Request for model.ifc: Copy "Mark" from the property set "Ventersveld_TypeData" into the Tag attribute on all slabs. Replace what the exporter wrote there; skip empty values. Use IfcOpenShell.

First a look at what the model holds.

```python
import ifcopenshell
import ifcopenshell.util.element

model = ifcopenshell.open("model.ifc")
print(model.schema)
slabs = model.by_type("IfcSlab")
print(len(slabs), "slabs")
for e in slabs[:8]:
    source = ifcopenshell.util.element.get_pset(e, "Ventersveld_TypeData", "Mark")
    target = e.Tag
    print(e.id(), repr(source), repr(target), sep=" | ")
```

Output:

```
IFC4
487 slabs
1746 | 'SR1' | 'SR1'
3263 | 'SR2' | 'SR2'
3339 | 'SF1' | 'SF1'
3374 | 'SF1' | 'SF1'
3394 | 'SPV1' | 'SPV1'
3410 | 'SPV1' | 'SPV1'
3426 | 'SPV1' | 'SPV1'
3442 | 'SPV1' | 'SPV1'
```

```python
import ifcopenshell
import ifcopenshell.util.element

model = ifcopenshell.open("model.ifc")

count = 0
for e in model.by_type("IfcSlab"):
    value = ifcopenshell.util.element.get_pset(e, "Ventersveld_TypeData", "Mark")
    current = e.Tag
    if not value or not value.strip() or current == value:
        continue
    e.Tag = value
    count += 1

print(count, "slabs updated")

model.write("model_edited.ifc")
```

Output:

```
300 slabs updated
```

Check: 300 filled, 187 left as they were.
